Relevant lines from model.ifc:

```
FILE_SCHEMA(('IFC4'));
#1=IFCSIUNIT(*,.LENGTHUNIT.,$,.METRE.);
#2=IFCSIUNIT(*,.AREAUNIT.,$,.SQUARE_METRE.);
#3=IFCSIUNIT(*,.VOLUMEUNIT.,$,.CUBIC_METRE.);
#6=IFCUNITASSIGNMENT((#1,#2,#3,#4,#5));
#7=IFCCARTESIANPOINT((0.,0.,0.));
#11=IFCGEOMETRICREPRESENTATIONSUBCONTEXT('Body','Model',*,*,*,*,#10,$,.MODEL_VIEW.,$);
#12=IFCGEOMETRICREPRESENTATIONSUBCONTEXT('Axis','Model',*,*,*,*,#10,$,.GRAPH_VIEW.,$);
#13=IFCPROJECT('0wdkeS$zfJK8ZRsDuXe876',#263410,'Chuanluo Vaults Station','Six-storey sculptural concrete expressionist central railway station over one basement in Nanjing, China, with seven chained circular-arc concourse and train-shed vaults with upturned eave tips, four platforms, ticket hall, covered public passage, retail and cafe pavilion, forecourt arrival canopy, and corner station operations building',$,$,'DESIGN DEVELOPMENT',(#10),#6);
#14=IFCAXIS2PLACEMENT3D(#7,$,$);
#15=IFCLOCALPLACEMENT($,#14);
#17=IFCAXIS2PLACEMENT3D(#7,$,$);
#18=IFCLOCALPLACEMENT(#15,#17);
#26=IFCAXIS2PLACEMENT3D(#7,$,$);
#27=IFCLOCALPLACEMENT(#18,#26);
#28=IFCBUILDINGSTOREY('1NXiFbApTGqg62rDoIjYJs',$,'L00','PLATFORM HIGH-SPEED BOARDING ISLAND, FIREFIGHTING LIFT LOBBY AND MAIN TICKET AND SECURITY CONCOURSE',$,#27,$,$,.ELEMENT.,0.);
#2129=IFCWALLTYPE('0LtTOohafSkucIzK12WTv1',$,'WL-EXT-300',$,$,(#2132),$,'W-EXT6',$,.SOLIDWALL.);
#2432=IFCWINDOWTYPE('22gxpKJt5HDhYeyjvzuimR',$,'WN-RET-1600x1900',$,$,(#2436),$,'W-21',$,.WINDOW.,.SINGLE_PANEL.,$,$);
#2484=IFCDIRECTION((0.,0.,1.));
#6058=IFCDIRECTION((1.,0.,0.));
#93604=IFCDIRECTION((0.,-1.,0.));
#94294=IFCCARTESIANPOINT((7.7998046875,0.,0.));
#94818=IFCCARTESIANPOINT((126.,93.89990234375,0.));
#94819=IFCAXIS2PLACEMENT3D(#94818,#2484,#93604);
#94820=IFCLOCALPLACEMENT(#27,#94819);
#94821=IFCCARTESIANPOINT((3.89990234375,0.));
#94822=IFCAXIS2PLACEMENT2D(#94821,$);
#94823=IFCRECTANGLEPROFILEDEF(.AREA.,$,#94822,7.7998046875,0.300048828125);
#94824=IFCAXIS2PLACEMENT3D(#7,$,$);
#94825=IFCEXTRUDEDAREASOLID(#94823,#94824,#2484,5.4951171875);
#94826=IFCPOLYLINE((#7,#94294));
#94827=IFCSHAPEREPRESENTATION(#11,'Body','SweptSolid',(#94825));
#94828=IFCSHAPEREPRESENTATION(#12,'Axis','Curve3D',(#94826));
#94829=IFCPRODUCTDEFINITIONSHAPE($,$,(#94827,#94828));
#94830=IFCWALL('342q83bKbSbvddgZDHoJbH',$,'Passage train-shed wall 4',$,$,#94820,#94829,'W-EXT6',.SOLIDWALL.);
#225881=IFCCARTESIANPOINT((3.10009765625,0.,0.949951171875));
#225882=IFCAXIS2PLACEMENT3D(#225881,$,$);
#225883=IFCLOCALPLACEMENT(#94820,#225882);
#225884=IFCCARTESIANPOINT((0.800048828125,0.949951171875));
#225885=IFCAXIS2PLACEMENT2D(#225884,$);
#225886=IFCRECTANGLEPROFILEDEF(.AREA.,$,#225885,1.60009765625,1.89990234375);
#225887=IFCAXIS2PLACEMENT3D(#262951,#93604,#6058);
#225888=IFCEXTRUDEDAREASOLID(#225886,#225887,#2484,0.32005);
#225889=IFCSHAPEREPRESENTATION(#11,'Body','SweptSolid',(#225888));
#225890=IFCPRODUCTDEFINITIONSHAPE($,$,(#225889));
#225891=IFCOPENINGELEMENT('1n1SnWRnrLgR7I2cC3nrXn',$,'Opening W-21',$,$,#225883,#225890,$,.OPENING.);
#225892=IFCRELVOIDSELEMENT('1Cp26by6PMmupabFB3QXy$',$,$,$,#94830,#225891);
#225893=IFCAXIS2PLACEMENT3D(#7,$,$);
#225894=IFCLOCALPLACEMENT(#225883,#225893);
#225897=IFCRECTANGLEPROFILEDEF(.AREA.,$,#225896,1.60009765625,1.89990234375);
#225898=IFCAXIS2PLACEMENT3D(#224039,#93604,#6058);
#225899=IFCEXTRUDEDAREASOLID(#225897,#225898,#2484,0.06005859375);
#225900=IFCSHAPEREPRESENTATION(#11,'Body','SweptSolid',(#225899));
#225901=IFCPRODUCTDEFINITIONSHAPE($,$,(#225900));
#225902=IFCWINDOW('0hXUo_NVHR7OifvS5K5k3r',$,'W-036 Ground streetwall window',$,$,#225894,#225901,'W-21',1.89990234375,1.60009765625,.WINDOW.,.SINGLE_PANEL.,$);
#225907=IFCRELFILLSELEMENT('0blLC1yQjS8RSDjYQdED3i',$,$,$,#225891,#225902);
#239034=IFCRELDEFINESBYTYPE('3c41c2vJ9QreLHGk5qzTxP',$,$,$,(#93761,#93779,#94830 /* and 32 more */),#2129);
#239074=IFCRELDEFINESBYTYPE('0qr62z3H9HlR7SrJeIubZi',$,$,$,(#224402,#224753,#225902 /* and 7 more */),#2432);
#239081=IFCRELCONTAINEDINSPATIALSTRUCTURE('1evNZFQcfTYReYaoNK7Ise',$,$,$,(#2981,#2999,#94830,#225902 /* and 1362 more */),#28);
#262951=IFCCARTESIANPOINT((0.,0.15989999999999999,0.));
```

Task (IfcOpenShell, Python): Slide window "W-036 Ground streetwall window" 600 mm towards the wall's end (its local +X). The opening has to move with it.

```python
import ifcopenshell
import ifcopenshell.api.geometry
import ifcopenshell.util.placement

model = ifcopenshell.open("model.ifc")

window = model.by_id(225902)
opening = window.FillsVoids[0].RelatingOpeningElement
wall = opening.VoidsElements[0].RelatingBuildingElement

wall_matrix = ifcopenshell.util.placement.get_local_placement(wall.ObjectPlacement)
shift = wall_matrix[:3, 0] * 0.6
before = ifcopenshell.util.placement.get_local_placement(window.ObjectPlacement)[:3, 3].copy()

# The window is placed relative to its opening, so it follows when the opening moves.
matrix = ifcopenshell.util.placement.get_local_placement(opening.ObjectPlacement)
matrix[:3, 3] += shift
ifcopenshell.api.geometry.edit_object_placement(
    model, product=opening, matrix=matrix, is_si=False, should_transform_children=True
)

after = ifcopenshell.util.placement.get_local_placement(window.ObjectPlacement)[:3, 3]
print("window moved by", (after - before).round(3) + 0.0)

model.write("model-out.ifc")
```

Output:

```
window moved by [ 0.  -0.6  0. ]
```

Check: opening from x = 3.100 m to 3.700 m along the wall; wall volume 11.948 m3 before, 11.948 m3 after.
